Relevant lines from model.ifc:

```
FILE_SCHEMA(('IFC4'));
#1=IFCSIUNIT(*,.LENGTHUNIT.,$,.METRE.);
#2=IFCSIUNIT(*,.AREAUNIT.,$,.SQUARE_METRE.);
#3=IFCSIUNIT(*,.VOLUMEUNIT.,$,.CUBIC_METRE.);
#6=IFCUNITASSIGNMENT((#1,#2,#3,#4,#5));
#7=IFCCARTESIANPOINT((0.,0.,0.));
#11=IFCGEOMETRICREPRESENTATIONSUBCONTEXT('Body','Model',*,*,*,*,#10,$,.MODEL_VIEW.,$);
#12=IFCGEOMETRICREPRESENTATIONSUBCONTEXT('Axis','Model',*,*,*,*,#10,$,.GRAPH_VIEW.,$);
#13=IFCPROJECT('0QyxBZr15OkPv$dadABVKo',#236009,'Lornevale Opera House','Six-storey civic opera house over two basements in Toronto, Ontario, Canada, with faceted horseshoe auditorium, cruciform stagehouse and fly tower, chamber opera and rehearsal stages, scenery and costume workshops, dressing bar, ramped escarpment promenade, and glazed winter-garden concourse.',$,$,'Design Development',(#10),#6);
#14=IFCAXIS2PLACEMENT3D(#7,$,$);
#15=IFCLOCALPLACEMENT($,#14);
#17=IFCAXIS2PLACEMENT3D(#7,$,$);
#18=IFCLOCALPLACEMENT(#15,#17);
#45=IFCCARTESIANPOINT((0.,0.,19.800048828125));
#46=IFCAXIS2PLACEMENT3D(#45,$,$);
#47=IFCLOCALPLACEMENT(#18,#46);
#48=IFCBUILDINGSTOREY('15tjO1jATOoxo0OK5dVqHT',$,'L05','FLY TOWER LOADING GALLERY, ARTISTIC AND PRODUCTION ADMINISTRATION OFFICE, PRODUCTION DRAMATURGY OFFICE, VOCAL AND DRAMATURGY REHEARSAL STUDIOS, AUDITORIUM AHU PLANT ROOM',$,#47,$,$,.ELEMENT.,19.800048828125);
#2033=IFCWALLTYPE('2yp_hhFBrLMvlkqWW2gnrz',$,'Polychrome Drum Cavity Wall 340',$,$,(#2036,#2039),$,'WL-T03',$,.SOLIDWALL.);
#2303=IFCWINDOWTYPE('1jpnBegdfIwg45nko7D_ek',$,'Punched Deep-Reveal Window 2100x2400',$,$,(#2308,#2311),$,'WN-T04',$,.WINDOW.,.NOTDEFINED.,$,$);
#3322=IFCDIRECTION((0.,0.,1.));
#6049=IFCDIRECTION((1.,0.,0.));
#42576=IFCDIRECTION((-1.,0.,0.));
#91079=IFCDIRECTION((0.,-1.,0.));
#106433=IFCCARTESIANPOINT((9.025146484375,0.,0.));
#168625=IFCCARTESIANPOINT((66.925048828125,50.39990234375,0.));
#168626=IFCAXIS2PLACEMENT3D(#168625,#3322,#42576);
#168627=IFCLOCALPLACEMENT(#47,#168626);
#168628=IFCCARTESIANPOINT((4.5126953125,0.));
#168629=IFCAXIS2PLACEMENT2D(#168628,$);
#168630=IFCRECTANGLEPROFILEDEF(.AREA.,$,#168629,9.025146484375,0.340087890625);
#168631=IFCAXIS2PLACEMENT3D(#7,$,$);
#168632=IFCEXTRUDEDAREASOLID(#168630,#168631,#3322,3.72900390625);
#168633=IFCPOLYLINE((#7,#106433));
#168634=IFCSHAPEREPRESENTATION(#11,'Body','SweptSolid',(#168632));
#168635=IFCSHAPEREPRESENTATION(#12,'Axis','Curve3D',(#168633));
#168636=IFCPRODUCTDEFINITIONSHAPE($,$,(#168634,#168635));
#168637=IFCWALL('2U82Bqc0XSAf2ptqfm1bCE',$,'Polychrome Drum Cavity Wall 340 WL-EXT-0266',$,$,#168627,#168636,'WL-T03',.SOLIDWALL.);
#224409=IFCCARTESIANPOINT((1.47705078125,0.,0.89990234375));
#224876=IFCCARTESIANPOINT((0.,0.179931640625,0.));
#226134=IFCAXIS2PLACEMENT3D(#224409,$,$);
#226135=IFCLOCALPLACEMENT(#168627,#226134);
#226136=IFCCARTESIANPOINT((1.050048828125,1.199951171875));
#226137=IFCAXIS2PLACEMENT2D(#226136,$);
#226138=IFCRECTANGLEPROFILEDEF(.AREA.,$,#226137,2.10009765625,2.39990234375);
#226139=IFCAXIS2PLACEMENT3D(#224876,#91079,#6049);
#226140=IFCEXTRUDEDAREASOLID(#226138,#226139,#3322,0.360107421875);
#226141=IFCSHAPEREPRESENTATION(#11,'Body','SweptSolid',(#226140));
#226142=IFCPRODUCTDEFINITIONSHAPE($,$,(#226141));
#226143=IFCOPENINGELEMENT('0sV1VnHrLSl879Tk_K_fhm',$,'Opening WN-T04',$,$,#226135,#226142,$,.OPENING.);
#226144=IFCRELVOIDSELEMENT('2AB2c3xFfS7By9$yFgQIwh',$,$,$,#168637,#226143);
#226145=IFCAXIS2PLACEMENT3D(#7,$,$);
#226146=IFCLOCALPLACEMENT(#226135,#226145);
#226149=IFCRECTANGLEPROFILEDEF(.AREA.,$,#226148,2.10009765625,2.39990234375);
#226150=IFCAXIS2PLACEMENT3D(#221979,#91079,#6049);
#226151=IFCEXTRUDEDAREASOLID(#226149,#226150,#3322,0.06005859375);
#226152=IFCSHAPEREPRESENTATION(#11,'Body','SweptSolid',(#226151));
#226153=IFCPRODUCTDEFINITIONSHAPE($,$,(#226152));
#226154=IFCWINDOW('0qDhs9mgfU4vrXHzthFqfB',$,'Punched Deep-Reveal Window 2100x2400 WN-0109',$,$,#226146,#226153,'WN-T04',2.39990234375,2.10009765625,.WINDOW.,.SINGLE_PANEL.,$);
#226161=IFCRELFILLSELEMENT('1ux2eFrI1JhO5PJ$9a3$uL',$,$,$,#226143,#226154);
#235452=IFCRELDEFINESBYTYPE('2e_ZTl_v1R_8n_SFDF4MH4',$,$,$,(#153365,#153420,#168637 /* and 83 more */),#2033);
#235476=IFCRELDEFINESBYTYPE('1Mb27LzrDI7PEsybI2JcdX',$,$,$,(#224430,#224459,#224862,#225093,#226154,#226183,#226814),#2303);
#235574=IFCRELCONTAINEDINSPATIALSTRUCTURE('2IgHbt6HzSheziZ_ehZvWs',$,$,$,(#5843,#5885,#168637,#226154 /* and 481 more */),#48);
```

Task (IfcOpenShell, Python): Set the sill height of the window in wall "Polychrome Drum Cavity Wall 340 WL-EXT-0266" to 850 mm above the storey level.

```python
import numpy as np
import ifcopenshell
import ifcopenshell.api.geometry
import ifcopenshell.geom
import ifcopenshell.util.element
import ifcopenshell.util.placement
import ifcopenshell.util.shape
import ifcopenshell.util.unit

model = ifcopenshell.open("model.ifc")
unit_scale = ifcopenshell.util.unit.calculate_unit_scale(model)

window = model.by_guid("0qDhs9mgfU4vrXHzthFqfB")
opening = window.FillsVoids[0].RelatingOpeningElement
storey = ifcopenshell.util.element.get_container(window, ifc_class="IfcBuildingStorey")
level = ifcopenshell.util.placement.get_local_placement(storey.ObjectPlacement)[2, 3]

# The opening's origin need not be at the sill, so measure its lowest point.
shape = ifcopenshell.geom.create_shape(ifcopenshell.geom.settings(), opening)
bottom = ifcopenshell.util.shape.get_shape_bottom_elevation(shape, shape.geometry) / unit_scale
dz = level + 0.85 - bottom

shift = np.array([0.0, 0.0, dz])
# The window is placed relative to its opening, so it follows when the opening moves.
matrix = ifcopenshell.util.placement.get_local_placement(opening.ObjectPlacement)
matrix[:3, 3] += shift
ifcopenshell.api.geometry.edit_object_placement(
    model, product=opening, matrix=matrix, is_si=False, should_transform_children=True
)

print(f"moved by {dz * unit_scale:+.3f} m")

model.write("model_rev.ifc")
```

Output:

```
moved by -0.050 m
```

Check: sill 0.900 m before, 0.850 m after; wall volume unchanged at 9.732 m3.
